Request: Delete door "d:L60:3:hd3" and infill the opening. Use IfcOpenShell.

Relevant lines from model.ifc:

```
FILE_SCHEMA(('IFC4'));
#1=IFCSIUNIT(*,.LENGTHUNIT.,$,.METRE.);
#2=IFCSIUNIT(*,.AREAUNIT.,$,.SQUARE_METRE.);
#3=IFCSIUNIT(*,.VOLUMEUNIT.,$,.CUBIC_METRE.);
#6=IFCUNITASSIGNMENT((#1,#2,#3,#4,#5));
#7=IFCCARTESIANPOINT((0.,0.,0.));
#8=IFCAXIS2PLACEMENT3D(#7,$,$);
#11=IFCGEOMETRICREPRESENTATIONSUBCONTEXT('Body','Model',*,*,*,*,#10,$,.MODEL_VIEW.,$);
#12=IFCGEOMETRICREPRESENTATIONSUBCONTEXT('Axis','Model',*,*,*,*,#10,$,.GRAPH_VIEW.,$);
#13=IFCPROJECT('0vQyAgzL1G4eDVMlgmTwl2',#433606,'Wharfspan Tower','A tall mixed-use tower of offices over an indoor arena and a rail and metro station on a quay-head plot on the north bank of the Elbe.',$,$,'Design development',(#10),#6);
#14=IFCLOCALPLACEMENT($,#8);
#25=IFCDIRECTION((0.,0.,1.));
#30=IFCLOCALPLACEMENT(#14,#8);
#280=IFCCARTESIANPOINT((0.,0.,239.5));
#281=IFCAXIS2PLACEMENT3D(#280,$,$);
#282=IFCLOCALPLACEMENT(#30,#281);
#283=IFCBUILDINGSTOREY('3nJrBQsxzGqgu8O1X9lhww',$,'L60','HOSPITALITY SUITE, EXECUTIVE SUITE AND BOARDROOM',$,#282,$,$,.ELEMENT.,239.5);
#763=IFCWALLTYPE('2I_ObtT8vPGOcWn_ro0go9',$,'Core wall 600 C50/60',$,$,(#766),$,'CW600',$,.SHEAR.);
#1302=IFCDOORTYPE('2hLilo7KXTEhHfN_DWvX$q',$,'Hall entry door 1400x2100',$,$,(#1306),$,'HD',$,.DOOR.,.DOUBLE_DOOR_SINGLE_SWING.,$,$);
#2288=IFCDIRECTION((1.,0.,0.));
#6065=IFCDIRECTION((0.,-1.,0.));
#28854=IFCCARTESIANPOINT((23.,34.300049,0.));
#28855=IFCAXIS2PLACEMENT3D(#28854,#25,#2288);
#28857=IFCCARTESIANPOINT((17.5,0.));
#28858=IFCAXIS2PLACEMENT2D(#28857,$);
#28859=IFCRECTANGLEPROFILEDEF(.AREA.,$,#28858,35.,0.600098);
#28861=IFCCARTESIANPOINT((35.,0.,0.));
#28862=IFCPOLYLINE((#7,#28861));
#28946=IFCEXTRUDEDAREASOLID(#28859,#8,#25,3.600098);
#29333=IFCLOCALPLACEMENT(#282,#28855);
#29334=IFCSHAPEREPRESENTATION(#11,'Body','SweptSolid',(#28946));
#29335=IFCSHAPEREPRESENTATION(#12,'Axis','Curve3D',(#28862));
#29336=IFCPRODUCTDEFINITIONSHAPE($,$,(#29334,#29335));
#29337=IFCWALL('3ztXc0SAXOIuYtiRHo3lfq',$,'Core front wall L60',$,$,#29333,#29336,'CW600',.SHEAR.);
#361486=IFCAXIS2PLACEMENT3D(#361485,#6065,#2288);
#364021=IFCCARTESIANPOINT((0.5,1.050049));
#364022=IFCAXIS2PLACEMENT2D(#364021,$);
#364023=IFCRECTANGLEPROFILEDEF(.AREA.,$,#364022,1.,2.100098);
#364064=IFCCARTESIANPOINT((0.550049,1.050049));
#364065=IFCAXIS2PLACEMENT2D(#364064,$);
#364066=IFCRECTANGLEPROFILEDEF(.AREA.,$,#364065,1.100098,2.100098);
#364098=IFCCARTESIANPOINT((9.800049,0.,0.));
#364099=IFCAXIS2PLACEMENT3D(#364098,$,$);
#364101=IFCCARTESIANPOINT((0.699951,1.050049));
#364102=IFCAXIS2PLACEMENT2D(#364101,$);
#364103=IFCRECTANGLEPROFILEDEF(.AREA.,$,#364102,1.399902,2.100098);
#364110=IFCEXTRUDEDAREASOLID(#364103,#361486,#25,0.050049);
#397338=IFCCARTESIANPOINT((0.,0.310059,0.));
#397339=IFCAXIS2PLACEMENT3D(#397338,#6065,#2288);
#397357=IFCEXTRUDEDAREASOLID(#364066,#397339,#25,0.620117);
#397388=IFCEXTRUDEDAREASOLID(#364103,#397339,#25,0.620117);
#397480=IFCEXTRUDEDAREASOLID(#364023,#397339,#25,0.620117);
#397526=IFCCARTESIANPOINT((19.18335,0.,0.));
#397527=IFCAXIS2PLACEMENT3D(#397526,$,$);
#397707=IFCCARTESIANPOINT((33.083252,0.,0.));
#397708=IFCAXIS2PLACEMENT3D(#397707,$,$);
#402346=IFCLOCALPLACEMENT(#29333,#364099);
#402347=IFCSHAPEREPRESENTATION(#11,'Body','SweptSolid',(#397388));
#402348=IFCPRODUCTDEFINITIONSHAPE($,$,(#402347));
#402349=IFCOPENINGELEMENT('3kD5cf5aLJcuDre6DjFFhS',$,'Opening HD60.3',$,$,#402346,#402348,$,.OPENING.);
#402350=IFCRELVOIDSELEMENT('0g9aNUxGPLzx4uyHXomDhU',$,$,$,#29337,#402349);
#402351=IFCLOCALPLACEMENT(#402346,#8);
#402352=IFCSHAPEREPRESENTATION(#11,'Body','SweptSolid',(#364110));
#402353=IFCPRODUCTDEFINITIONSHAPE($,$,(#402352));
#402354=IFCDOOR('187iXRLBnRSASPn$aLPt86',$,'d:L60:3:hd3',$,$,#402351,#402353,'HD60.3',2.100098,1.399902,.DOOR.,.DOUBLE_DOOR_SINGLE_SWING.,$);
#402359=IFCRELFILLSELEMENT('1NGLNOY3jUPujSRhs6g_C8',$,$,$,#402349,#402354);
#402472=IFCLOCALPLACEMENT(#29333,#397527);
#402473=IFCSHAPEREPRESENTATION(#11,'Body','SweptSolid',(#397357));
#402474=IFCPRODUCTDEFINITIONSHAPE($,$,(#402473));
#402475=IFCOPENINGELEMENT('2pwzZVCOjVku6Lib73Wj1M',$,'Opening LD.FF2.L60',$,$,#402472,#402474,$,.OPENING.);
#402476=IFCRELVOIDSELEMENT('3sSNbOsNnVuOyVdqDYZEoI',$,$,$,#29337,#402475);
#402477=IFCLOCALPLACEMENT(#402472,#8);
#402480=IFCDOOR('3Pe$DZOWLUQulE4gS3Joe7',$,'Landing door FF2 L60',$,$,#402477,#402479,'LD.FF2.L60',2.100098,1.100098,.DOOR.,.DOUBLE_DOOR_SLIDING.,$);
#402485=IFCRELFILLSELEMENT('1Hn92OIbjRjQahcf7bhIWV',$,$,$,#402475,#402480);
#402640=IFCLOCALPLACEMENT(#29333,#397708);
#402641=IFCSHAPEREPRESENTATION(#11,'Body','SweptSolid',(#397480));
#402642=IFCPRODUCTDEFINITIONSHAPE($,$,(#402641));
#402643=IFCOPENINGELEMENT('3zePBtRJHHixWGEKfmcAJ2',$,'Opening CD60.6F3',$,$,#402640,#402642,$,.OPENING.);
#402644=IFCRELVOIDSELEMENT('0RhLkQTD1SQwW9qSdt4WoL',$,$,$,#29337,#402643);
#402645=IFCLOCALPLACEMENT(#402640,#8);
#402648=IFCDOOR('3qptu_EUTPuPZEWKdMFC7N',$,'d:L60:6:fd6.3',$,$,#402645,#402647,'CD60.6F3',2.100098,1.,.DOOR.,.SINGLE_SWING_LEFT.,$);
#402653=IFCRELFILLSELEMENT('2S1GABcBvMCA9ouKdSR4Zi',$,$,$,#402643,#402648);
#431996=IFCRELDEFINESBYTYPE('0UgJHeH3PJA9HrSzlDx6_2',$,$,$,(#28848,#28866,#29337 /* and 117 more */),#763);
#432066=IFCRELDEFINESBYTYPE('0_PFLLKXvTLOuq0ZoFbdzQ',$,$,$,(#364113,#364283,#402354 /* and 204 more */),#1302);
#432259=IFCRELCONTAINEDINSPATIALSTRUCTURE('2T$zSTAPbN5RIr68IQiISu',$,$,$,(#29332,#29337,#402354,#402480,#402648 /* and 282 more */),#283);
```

```python
import ifcopenshell
import ifcopenshell.api.feature
import ifcopenshell.api.root
import ifcopenshell.geom
import ifcopenshell.util.shape

model = ifcopenshell.open("model.ifc")
settings = ifcopenshell.geom.settings()


def volume(element):
    """Net volume in cubic metres, openings subtracted."""
    shape = ifcopenshell.geom.create_shape(settings, element)
    return ifcopenshell.util.shape.get_volume(shape.geometry)


door = model.by_id(402354)
opening = door.FillsVoids[0].RelatingOpeningElement
wall = opening.VoidsElements[0].RelatingBuildingElement
before = volume(wall)

ifcopenshell.api.root.remove_product(model, product=door)
ifcopenshell.api.feature.remove_feature(model, feature=opening)

after = volume(wall)

print(f"wall volume {before:.3f} -> {after:.3f} m3")

model.write("model_edited.ifc")
```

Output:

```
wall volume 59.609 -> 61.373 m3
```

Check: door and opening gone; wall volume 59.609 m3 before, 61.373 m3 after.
